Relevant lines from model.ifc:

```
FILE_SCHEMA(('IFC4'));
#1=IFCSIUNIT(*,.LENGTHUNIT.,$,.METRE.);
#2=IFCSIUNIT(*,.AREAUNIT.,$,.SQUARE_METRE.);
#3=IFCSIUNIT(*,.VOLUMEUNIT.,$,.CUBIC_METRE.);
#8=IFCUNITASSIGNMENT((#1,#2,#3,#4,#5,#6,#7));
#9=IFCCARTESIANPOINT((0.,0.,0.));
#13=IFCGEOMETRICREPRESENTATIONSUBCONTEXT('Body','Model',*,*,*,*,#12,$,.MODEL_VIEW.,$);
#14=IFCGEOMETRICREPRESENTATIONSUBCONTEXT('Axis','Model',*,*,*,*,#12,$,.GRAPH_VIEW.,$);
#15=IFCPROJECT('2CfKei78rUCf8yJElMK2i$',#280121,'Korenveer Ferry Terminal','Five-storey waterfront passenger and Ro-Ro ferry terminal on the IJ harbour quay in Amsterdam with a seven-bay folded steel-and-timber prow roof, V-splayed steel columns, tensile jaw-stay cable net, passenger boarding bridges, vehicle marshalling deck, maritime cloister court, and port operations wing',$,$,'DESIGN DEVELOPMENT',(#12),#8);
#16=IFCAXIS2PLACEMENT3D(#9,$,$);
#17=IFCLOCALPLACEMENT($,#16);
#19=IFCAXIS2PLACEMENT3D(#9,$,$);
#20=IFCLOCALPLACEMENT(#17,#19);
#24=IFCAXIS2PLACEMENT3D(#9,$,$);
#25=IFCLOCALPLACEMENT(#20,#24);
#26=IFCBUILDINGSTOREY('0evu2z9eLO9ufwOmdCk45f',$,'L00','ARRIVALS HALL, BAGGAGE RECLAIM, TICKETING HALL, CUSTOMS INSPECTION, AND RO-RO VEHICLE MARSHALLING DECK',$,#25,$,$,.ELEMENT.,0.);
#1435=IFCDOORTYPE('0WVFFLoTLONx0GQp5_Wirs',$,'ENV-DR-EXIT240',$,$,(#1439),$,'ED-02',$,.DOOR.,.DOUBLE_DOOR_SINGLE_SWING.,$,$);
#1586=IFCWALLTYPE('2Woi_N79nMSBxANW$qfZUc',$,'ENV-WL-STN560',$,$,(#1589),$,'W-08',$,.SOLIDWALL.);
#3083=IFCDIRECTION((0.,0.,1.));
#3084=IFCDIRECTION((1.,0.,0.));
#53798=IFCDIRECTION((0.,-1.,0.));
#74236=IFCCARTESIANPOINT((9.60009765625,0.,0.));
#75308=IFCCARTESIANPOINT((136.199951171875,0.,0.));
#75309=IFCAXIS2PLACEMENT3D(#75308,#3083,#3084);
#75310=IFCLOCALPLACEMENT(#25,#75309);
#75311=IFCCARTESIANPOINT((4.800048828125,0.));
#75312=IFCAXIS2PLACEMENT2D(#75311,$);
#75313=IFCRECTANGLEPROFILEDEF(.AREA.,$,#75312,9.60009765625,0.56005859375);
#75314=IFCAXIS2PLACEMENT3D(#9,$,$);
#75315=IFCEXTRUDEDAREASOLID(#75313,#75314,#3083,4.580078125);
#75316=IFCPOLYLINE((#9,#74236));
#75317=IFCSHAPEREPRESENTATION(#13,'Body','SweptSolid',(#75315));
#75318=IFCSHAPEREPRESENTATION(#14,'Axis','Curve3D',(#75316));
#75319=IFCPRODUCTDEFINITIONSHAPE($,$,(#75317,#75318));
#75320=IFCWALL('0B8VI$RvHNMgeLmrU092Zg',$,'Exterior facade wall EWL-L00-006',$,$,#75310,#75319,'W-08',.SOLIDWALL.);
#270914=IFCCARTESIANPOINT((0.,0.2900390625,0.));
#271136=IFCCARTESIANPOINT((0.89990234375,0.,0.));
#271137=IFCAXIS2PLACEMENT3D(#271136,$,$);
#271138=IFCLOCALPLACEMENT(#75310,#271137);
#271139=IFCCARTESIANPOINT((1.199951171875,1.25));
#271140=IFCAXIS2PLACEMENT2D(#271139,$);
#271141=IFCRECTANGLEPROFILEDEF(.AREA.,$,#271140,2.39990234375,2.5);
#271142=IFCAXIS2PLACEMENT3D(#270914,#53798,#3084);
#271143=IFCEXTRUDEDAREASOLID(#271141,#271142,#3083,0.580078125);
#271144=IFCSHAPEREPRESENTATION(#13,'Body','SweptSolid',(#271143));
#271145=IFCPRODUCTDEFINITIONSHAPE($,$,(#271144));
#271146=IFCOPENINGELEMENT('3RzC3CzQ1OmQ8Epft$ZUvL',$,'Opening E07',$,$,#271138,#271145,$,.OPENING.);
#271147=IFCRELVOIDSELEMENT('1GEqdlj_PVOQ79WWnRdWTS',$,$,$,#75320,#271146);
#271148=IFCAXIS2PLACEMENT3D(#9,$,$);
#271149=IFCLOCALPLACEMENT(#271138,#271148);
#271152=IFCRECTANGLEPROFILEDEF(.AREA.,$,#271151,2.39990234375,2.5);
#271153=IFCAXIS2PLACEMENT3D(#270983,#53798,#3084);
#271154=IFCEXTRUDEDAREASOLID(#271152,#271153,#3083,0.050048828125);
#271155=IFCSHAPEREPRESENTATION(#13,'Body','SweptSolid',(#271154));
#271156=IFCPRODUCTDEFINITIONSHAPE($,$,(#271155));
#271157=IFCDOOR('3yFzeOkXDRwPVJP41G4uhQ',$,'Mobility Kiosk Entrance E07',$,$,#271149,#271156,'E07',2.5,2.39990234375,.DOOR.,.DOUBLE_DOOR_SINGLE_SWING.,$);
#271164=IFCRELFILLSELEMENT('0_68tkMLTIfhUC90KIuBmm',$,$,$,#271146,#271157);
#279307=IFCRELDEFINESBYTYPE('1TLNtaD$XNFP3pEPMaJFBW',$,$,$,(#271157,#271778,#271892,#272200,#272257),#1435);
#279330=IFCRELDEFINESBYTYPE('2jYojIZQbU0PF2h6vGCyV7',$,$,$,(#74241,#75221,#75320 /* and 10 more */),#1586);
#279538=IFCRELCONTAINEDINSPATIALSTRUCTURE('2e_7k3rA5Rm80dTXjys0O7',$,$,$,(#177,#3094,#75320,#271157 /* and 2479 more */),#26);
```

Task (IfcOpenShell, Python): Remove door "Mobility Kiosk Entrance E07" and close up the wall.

```python
import ifcopenshell
import ifcopenshell.api.feature
import ifcopenshell.api.root
import ifcopenshell.geom
import ifcopenshell.util.shape

model = ifcopenshell.open("model.ifc")
settings = ifcopenshell.geom.settings()


def volume(element):
    """Net volume in cubic metres, openings subtracted."""
    shape = ifcopenshell.geom.create_shape(settings, element)
    return ifcopenshell.util.shape.get_volume(shape.geometry)


door = model.by_guid("3yFzeOkXDRwPVJP41G4uhQ")
opening = door.FillsVoids[0].RelatingOpeningElement
wall = opening.VoidsElements[0].RelatingBuildingElement
before = volume(wall)

ifcopenshell.api.root.remove_product(model, product=door)
ifcopenshell.api.feature.remove_feature(model, feature=opening)

after = volume(wall)

print(f"wall volume {before:.3f} -> {after:.3f} m3")

model.write("model_updated.ifc")
```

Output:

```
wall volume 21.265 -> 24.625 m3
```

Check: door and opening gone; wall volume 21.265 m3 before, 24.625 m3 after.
